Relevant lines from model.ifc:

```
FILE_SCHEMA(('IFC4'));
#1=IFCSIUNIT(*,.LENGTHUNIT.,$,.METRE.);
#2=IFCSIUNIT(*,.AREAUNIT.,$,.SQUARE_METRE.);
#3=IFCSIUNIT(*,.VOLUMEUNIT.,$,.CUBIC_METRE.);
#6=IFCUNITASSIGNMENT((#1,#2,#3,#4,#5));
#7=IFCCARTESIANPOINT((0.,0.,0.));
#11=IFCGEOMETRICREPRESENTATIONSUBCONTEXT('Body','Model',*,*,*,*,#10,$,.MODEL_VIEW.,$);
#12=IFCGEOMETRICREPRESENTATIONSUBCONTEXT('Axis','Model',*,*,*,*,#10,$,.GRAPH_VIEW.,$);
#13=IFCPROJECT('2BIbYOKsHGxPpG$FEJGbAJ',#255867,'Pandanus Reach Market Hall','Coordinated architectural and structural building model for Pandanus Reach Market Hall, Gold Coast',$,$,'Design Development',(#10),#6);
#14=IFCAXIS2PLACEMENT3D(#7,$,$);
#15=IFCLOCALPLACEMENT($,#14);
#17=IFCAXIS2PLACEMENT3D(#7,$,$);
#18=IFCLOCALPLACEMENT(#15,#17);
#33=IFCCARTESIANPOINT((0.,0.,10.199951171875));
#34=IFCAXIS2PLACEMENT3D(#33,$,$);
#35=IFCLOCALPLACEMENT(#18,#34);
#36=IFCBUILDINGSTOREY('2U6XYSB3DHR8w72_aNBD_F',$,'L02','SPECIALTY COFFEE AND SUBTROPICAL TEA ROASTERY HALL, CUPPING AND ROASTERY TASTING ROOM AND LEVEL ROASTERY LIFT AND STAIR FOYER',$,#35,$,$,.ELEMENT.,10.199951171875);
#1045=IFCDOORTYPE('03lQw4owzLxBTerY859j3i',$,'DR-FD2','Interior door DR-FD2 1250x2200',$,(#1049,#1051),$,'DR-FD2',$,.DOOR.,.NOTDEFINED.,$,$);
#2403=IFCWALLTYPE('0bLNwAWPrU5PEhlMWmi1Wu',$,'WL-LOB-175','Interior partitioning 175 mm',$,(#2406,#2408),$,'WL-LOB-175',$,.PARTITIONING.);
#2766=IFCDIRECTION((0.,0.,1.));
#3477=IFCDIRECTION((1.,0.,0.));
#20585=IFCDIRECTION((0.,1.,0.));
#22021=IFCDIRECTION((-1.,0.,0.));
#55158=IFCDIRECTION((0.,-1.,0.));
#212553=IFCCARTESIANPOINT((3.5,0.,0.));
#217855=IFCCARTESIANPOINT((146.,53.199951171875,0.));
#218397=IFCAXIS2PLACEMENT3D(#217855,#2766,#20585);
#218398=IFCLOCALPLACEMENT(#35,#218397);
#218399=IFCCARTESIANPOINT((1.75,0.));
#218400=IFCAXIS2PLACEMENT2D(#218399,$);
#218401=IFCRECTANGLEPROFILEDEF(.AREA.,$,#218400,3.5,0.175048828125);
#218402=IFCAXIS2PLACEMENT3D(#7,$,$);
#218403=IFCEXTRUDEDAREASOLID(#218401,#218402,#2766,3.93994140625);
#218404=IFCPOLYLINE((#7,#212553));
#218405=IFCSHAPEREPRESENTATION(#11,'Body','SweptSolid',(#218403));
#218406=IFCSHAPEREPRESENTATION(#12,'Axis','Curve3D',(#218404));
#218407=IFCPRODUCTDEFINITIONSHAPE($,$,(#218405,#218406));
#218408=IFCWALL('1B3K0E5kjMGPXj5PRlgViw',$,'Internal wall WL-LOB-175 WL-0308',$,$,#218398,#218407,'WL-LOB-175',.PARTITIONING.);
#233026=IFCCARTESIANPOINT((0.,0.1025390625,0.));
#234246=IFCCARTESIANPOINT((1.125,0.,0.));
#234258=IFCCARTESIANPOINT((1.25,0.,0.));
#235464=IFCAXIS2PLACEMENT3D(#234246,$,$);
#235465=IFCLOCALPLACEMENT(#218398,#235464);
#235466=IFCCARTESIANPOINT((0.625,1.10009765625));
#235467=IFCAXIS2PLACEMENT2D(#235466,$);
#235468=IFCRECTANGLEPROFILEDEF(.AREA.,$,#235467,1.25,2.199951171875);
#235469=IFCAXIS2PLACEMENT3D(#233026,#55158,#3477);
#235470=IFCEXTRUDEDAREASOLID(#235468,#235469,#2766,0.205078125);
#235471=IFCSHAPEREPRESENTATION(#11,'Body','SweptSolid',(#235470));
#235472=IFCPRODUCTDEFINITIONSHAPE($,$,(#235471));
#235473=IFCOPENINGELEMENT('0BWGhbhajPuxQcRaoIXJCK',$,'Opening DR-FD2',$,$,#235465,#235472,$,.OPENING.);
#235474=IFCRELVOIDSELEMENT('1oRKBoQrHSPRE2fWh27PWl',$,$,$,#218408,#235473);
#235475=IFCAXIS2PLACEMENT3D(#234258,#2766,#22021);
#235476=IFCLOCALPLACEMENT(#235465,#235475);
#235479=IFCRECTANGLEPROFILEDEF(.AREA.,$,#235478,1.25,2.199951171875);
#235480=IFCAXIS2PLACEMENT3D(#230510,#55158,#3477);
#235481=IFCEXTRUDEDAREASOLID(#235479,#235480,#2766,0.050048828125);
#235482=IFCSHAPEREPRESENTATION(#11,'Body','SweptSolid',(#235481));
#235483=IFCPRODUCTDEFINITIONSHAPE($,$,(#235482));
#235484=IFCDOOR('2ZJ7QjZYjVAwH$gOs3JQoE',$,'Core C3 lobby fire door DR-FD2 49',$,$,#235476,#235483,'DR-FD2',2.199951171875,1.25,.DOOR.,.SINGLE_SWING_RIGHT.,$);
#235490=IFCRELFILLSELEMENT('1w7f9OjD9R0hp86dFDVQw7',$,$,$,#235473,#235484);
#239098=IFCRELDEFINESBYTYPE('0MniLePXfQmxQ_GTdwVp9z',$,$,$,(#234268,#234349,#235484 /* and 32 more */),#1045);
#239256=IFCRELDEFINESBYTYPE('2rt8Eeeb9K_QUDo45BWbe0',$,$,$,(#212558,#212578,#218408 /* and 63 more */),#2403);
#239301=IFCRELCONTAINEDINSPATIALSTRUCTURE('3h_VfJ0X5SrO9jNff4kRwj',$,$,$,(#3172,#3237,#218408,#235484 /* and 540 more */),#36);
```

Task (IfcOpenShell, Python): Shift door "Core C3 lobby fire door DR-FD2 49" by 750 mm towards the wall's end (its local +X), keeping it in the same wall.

```python
import ifcopenshell
import ifcopenshell.api.geometry
import ifcopenshell.util.placement

model = ifcopenshell.open("model.ifc")

door = model.by_guid("2ZJ7QjZYjVAwH$gOs3JQoE")
opening = door.FillsVoids[0].RelatingOpeningElement
wall = opening.VoidsElements[0].RelatingBuildingElement

wall_matrix = ifcopenshell.util.placement.get_local_placement(wall.ObjectPlacement)
shift = wall_matrix[:3, 0] * 0.75
before = ifcopenshell.util.placement.get_local_placement(door.ObjectPlacement)[:3, 3].copy()

# The door is placed relative to its opening, so it follows when the opening moves.
matrix = ifcopenshell.util.placement.get_local_placement(opening.ObjectPlacement)
matrix[:3, 3] += shift
ifcopenshell.api.geometry.edit_object_placement(
    model, product=opening, matrix=matrix, is_si=False, should_transform_children=True
)

after = ifcopenshell.util.placement.get_local_placement(door.ObjectPlacement)[:3, 3]
print("door moved by", (after - before).round(3) + 0.0)

model.write("model_updated.ifc")
```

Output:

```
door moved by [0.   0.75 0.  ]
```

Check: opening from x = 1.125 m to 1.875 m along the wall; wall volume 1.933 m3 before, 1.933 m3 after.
